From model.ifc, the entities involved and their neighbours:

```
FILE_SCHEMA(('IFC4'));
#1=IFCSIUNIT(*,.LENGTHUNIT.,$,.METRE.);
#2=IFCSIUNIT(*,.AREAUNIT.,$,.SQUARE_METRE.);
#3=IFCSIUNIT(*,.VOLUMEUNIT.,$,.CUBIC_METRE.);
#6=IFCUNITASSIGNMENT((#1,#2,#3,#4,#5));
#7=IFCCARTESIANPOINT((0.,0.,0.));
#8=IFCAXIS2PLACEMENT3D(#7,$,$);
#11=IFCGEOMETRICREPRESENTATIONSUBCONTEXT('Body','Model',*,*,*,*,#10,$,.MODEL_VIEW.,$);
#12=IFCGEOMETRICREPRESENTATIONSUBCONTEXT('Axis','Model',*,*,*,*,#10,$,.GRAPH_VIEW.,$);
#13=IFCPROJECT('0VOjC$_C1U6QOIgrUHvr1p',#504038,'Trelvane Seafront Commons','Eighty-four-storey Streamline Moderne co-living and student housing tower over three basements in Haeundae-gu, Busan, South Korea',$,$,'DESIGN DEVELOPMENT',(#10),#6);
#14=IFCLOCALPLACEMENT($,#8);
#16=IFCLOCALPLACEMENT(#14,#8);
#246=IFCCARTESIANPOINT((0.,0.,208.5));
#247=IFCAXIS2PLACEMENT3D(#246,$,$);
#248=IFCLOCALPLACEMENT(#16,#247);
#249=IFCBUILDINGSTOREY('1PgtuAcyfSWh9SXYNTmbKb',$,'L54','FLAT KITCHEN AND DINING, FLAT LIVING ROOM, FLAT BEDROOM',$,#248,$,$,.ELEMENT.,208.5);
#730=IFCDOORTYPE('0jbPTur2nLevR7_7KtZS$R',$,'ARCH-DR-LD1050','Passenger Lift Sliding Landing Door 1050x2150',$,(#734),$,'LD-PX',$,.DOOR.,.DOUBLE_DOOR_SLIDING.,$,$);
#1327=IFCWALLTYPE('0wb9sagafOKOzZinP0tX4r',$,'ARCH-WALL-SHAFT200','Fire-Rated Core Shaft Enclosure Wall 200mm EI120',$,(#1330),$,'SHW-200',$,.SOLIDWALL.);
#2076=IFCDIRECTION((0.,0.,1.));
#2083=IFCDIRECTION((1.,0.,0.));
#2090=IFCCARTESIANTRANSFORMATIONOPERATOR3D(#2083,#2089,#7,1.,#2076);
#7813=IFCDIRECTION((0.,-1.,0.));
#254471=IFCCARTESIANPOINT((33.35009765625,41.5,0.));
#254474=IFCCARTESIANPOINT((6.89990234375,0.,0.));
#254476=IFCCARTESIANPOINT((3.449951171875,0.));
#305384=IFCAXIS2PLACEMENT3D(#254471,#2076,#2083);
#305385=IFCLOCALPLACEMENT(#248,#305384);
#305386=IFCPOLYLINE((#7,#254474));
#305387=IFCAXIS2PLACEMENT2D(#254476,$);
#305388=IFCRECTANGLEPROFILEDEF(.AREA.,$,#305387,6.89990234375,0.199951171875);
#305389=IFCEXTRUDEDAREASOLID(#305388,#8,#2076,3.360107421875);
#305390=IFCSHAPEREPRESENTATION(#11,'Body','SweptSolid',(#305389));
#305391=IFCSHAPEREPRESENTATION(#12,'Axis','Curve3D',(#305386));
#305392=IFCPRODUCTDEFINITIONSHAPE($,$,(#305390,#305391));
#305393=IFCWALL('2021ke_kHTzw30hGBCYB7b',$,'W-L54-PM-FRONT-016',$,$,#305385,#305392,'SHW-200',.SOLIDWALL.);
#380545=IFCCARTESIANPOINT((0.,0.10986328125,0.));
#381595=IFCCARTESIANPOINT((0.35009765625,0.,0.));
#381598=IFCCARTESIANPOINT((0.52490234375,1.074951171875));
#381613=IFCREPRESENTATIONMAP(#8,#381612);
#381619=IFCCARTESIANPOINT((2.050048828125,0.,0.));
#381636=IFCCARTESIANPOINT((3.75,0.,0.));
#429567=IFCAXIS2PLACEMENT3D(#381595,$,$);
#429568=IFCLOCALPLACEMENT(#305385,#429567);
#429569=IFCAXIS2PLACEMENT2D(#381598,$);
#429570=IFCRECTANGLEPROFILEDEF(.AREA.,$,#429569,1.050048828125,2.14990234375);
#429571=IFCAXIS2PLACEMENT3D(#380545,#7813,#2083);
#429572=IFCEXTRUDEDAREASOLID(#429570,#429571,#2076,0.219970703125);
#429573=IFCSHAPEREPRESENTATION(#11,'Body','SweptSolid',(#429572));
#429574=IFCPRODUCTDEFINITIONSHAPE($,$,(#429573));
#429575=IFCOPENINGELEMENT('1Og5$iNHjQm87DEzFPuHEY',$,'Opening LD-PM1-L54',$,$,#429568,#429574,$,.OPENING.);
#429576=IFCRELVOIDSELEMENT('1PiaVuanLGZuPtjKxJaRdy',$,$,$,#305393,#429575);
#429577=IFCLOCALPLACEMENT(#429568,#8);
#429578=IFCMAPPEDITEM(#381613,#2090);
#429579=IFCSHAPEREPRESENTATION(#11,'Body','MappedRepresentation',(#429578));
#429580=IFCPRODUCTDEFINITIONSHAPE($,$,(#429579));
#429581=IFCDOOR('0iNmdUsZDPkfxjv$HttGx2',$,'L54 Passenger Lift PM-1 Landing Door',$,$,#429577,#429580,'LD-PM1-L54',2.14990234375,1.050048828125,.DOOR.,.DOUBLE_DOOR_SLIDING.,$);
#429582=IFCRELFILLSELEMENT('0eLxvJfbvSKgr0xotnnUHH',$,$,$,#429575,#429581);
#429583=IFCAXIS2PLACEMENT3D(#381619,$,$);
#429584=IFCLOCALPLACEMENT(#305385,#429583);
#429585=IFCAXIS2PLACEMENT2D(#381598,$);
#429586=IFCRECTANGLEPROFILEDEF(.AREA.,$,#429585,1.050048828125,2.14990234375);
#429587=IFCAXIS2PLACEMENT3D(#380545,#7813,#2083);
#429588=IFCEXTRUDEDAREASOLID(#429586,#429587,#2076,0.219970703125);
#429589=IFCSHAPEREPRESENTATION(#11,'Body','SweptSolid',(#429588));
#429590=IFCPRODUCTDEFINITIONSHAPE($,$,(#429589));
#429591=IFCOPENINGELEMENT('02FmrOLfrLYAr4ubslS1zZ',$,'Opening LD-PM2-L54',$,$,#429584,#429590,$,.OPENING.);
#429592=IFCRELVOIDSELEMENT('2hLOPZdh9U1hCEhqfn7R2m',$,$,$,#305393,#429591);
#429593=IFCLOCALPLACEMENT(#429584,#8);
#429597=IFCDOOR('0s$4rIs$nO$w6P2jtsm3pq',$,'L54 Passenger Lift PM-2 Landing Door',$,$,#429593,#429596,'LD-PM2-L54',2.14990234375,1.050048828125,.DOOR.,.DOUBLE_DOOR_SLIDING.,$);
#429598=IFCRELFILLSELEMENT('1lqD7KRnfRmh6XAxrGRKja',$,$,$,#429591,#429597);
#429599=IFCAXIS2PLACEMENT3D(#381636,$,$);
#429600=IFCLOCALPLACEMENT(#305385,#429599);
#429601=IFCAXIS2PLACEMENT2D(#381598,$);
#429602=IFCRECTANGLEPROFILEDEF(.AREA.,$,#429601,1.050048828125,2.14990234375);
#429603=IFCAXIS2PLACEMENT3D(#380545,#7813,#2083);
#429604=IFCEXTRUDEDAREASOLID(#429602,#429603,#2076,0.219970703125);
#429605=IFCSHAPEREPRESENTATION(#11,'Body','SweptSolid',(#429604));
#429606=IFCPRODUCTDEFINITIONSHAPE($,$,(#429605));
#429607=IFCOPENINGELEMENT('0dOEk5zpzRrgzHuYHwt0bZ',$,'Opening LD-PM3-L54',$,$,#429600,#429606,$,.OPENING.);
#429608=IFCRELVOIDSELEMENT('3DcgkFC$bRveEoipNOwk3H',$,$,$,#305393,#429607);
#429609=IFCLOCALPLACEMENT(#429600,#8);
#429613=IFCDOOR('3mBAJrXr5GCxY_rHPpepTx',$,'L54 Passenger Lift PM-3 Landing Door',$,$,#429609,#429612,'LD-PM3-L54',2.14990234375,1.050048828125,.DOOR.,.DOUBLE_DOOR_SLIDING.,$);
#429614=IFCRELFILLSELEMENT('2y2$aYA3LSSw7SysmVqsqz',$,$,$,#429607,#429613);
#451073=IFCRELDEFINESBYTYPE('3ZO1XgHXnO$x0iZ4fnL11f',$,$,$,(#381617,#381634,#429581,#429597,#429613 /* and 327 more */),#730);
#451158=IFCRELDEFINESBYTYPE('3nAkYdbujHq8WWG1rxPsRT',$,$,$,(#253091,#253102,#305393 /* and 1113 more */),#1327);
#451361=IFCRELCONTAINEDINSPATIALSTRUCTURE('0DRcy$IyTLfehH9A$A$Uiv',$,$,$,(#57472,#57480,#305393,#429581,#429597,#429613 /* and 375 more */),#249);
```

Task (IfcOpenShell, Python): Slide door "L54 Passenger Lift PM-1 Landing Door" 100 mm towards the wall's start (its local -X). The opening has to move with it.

```python
import ifcopenshell
import ifcopenshell.api.geometry
import ifcopenshell.util.placement
import ifcopenshell.util.unit

model = ifcopenshell.open("model.ifc")
unit_scale = ifcopenshell.util.unit.calculate_unit_scale(model)

door = model.by_guid("0iNmdUsZDPkfxjv$HttGx2")
opening = door.FillsVoids[0].RelatingOpeningElement
wall = opening.VoidsElements[0].RelatingBuildingElement

wall_matrix = ifcopenshell.util.placement.get_local_placement(wall.ObjectPlacement)
shift = wall_matrix[:3, 0] * -0.1 / unit_scale
before = ifcopenshell.util.placement.get_local_placement(door.ObjectPlacement)[:3, 3].copy()

# The door is placed relative to its opening, so it follows when the opening moves.
matrix = ifcopenshell.util.placement.get_local_placement(opening.ObjectPlacement)
matrix[:3, 3] += shift
ifcopenshell.api.geometry.edit_object_placement(
    model, product=opening, matrix=matrix, is_si=False, should_transform_children=True
)

after = ifcopenshell.util.placement.get_local_placement(door.ObjectPlacement)[:3, 3]
print("door moved by", (after - before).round(3) + 0.0)

model.write("model_rev.ifc")
```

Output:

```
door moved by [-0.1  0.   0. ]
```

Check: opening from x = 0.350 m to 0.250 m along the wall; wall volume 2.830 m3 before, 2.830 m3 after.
